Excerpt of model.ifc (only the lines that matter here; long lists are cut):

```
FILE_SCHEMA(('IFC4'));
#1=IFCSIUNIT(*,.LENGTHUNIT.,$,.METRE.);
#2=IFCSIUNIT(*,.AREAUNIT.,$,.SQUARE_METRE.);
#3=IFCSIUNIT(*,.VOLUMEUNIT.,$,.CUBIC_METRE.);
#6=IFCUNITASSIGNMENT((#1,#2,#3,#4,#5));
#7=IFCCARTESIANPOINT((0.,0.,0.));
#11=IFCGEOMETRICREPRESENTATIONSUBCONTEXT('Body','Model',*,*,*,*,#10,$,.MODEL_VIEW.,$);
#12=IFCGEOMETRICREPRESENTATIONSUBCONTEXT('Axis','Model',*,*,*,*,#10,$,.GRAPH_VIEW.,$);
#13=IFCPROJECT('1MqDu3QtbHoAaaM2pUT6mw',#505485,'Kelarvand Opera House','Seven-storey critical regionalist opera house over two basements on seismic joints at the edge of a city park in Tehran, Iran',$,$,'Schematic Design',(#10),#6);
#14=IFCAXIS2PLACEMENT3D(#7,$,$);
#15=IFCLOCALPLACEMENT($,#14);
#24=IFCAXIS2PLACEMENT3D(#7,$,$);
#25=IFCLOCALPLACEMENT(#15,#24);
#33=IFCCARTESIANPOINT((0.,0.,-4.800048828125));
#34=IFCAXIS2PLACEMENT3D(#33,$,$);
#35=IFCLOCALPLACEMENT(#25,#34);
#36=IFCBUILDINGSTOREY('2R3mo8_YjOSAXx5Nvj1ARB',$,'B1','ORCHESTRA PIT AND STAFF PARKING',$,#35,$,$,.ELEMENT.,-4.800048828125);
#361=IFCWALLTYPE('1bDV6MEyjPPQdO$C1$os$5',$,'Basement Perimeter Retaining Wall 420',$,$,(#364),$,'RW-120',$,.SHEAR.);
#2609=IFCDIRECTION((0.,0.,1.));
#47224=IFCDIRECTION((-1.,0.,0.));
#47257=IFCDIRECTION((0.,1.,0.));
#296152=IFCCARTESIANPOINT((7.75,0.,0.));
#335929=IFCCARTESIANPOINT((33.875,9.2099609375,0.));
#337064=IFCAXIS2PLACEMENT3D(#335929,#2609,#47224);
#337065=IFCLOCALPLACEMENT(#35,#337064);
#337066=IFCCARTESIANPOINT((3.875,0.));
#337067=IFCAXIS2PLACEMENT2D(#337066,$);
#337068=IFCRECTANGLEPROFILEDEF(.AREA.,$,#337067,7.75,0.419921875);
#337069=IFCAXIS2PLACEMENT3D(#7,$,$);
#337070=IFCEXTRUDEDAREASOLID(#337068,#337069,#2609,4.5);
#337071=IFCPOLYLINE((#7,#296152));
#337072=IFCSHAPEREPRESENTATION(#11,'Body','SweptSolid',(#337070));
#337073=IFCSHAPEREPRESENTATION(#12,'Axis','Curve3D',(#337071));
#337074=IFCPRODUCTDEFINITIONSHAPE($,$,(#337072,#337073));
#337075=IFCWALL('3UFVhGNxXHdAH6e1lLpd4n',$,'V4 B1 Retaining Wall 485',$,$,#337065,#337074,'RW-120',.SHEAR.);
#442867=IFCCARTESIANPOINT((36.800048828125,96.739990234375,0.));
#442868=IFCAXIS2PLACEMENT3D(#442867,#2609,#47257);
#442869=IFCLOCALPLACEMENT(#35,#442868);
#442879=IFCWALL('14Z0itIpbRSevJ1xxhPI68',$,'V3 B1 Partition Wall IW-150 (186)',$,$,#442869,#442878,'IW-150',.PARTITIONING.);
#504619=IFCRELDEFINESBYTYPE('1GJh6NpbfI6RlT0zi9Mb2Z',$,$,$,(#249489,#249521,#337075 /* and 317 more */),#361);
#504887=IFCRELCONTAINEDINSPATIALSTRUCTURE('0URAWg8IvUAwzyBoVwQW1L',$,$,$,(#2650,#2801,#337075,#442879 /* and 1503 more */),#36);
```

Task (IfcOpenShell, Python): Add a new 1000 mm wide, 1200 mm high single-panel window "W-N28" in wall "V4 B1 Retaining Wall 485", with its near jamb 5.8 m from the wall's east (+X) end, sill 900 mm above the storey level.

```python
import numpy as np
import ifcopenshell
import ifcopenshell.api.feature
import ifcopenshell.api.geometry
import ifcopenshell.api.root
import ifcopenshell.api.spatial
import ifcopenshell.geom
import ifcopenshell.util.element
import ifcopenshell.util.placement
import ifcopenshell.util.representation
import ifcopenshell.util.shape
import ifcopenshell.util.unit

model = ifcopenshell.open("model.ifc")
unit_scale = ifcopenshell.util.unit.calculate_unit_scale(model)
settings = ifcopenshell.geom.settings()


def volume(element):
    """Net volume in cubic metres, openings subtracted."""
    shape = ifcopenshell.geom.create_shape(settings, element)
    return ifcopenshell.util.shape.get_volume(shape.geometry)


wall = model.by_id(337075)
storey = ifcopenshell.util.element.get_container(wall, ifc_class="IfcBuildingStorey")
context = ifcopenshell.util.representation.get_context(model, "Model", "Body", "MODEL_VIEW")
before = volume(wall)

width, height, from_end, sill = 1, 1.2, 5.8, 0.9  # metres

# The wall runs along its own X axis, and the end named is its -X end.
wall_shape = ifcopenshell.geom.create_shape(settings, wall)
x, y, z = ifcopenshell.util.shape.get_vertices(wall_shape.geometry).T
start = x.min() + from_end
face, thickness = float(y.min()), float(y.max() - y.min())
wall_matrix = ifcopenshell.util.placement.get_local_placement(wall.ObjectPlacement)
level = ifcopenshell.util.placement.get_local_placement(storey.ObjectPlacement)[2, 3]


def in_wall(x, y):
    """Placement at x, y metres in the wall's axes, at sill height."""
    matrix = wall_matrix.copy()
    matrix[:, 3] = wall_matrix @ np.array([x / unit_scale, y / unit_scale, 0.0, 1.0])
    matrix[2, 3] = level + sill / unit_scale
    return matrix


# Opening: a box that overshoots both wall faces by 50 mm.
opening = ifcopenshell.api.root.create_entity(model, ifc_class="IfcOpeningElement", predefined_type="OPENING")
box = ifcopenshell.api.geometry.add_wall_representation(
    model, context=context, length=width, height=height, thickness=thickness + 0.1
)
ifcopenshell.api.geometry.assign_representation(model, product=opening, representation=box)
ifcopenshell.api.geometry.edit_object_placement(model, product=opening, matrix=in_wall(start, face - 0.05), is_si=False)
ifcopenshell.api.feature.add_feature(model, feature=opening, element=wall)

window = ifcopenshell.api.root.create_entity(model, ifc_class="IfcWindow", name="W-N28", predefined_type="WINDOW")
window.OverallWidth, window.OverallHeight = width / unit_scale, height / unit_scale
window.PartitioningType = "SINGLE_PANEL"
body = ifcopenshell.api.geometry.add_window_representation(
    model,
    context=context,
    overall_width=window.OverallWidth,
    overall_height=window.OverallHeight,
    partition_type="SINGLE_PANEL",
)
ifcopenshell.api.geometry.assign_representation(model, product=window, representation=body)
ifcopenshell.api.spatial.assign_container(model, products=[window], relating_structure=storey)
ifcopenshell.api.feature.add_filling(model, opening=opening, element=window)

# Centre the window in the wall's thickness.
ifcopenshell.api.geometry.edit_object_placement(model, product=window, matrix=in_wall(start, face), is_si=False)
window_shape = ifcopenshell.geom.create_shape(settings, window)
depth = ifcopenshell.util.shape.get_vertices(window_shape.geometry)[:, 1]
offset = face + thickness / 2 - (depth.min() + depth.max()) / 2
ifcopenshell.api.geometry.edit_object_placement(model, product=window, matrix=in_wall(start, offset), is_si=False)

after = volume(wall)

print(f"wall volume {before:.3f} -> {after:.3f} m3")

model.write("model-out.ifc")
```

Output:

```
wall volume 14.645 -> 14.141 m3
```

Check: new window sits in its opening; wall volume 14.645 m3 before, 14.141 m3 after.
